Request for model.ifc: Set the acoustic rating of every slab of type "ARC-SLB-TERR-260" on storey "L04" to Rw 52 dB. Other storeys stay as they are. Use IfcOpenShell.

First a look at what the model holds.

```python
import ifcopenshell
import ifcopenshell.util.element

model = ifcopenshell.open("model.ifc")
print(model.schema)
storey = next(s for s in model.by_type("IfcBuildingStorey") if s.Name == "L04")
slabs = [e for e in ifcopenshell.util.element.get_decomposition(storey) if e.is_a("IfcSlab")]
seen = {}
for e in slabs:
    element_type = ifcopenshell.util.element.get_type(e)
    key = (element_type.Name if element_type != e and element_type else None, ifcopenshell.util.element.get_pset(e, "Pset_SlabCommon", "AcousticRating"))
    seen[key] = seen.get(key, 0) + 1
for (name, value), count in sorted(seen.items(), key=str):
    print(count, "x", name, "|", value)
```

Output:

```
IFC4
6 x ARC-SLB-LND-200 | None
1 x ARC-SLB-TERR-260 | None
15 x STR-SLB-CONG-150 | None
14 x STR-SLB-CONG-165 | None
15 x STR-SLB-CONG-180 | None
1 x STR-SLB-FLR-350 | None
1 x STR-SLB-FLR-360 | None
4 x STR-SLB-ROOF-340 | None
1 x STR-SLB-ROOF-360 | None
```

```python
import ifcopenshell
import ifcopenshell.api.pset
import ifcopenshell.util.element

model = ifcopenshell.open("model.ifc")

storey = next(s for s in model.by_type("IfcBuildingStorey") if s.Name == "L04")
slabs = [e for e in ifcopenshell.util.element.get_decomposition(storey) if e.is_a("IfcSlab")]

count = 0
for e in slabs:
    element_type = ifcopenshell.util.element.get_type(e)
    if element_type in (None, e) or element_type.Name != "ARC-SLB-TERR-260":
        continue
    # add_pset returns the element's existing set when there is one.
    pset = ifcopenshell.api.pset.add_pset(model, product=e, name="Pset_SlabCommon")
    ifcopenshell.api.pset.edit_pset(model, pset=pset, properties={"AcousticRating": "Rw 52 dB"})
    count += 1

print(count, "slabs updated")

model.write("model_updated.ifc")
```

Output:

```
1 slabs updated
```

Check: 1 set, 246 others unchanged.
